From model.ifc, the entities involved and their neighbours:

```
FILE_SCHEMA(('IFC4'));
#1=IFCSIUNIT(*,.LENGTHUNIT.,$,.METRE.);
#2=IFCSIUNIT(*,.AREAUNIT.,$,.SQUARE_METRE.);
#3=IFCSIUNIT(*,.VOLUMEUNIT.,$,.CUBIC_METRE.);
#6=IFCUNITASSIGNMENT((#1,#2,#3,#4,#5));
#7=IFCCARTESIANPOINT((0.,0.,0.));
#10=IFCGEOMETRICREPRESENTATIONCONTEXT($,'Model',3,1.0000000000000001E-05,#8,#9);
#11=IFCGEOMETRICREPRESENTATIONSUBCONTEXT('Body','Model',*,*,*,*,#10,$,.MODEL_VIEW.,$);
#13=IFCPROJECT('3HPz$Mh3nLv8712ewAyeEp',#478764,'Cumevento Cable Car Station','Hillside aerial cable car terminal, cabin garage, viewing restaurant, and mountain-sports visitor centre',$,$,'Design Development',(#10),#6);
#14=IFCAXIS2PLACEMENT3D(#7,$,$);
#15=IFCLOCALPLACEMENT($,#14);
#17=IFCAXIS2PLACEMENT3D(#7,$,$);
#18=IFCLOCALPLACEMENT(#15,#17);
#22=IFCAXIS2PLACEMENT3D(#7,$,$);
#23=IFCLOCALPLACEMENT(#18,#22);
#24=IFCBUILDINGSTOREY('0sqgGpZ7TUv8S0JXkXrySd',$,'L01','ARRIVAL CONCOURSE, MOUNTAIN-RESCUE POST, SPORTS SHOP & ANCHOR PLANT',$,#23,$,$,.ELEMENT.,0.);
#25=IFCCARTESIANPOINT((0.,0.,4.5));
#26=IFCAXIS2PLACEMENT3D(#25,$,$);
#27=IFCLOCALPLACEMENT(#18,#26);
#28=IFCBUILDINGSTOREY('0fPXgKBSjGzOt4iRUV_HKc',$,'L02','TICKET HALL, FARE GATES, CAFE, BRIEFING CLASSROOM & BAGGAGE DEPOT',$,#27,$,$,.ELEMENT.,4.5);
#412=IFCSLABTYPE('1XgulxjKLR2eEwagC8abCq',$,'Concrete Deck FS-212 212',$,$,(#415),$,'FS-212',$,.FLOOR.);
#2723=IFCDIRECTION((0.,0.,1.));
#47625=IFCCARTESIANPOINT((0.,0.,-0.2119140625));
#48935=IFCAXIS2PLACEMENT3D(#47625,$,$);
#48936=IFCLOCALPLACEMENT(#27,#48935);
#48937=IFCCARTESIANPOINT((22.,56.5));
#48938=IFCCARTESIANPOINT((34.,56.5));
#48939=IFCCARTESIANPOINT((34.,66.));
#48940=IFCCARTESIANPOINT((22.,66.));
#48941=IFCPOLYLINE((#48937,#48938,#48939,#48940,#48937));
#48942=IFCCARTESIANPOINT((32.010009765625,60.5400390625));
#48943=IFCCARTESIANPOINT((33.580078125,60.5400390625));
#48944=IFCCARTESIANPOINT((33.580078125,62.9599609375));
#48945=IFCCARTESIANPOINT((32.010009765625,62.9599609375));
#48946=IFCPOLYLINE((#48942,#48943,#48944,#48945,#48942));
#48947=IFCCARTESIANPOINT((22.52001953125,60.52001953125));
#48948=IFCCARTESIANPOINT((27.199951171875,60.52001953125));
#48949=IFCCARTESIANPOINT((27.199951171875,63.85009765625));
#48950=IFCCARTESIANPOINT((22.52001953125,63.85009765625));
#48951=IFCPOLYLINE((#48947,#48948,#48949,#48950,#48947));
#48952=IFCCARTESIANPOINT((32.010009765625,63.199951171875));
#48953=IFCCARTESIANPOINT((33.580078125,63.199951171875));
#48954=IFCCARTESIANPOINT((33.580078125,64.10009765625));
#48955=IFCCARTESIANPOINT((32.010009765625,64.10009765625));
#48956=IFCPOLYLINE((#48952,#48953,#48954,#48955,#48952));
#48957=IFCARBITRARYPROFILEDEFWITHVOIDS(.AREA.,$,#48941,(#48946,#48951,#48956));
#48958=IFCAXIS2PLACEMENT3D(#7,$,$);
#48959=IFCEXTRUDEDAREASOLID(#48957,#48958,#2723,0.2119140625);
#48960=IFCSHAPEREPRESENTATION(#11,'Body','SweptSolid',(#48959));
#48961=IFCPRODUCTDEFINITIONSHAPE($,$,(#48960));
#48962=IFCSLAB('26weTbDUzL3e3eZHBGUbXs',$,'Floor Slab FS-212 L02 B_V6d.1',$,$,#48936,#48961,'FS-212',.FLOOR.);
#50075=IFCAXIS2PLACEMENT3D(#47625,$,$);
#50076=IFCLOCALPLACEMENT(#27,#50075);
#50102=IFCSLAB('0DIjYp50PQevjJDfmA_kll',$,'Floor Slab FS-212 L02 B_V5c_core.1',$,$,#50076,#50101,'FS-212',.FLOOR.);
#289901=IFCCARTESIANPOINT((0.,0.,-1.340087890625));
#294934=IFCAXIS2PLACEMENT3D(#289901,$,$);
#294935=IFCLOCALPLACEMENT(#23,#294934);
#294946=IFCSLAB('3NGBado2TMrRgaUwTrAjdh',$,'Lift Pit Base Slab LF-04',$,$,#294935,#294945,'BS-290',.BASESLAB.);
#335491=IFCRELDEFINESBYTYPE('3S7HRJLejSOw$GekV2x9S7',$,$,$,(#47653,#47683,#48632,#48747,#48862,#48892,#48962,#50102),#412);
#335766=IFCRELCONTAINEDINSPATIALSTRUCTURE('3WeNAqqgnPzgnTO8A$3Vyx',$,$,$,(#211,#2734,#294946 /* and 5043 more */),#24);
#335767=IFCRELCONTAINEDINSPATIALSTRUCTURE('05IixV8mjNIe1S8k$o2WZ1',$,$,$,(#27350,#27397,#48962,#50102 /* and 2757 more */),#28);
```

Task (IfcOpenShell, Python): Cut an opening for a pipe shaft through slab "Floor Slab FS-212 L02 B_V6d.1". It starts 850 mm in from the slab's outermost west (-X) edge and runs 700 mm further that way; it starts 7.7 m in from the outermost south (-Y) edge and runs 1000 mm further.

```python
import numpy as np
import ifcopenshell
import ifcopenshell.api.feature
import ifcopenshell.api.geometry
import ifcopenshell.api.root
import ifcopenshell.geom
import ifcopenshell.util.placement
import ifcopenshell.util.representation
import ifcopenshell.util.shape
import ifcopenshell.util.unit

model = ifcopenshell.open("model.ifc")
unit_scale = ifcopenshell.util.unit.calculate_unit_scale(model)
settings = ifcopenshell.geom.settings()


def volume(element):
    """Net volume in cubic metres, openings subtracted."""
    shape = ifcopenshell.geom.create_shape(settings, element)
    return ifcopenshell.util.shape.get_volume(shape.geometry)


slab = model.by_guid("26weTbDUzL3e3eZHBGUbXs")
before = volume(slab)

# Extent in the slab's own axes, in metres. The edges named are its -X and -Y sides.
slab_shape = ifcopenshell.geom.create_shape(settings, slab)
vertices = ifcopenshell.util.shape.get_vertices(slab_shape.geometry)
x_min, y_min, bottom = vertices.min(axis=0)
top = vertices[:, 2].max()

opening = ifcopenshell.api.root.create_entity(model, ifc_class="IfcOpeningElement", name="Pipe shaft opening", predefined_type="OPENING")
context = ifcopenshell.util.representation.get_context(model, "Model", "Body", "MODEL_VIEW")
width, depth = 0.7, 1
outline = [(0.0, 0.0), (width, 0.0), (width, depth), (0.0, depth), (0.0, 0.0)]
# Overshoot both faces by 50 mm so the cut is clean.
shape = ifcopenshell.api.geometry.add_slab_representation(
    model, context=context, depth=top - bottom + 0.1, polyline=outline
)
ifcopenshell.api.geometry.assign_representation(model, product=opening, representation=shape)

matrix = ifcopenshell.util.placement.get_local_placement(slab.ObjectPlacement)
matrix[:, 3] = matrix @ np.append(np.array([x_min + 0.85, y_min + 7.7, bottom - 0.05]) / unit_scale, 1.0)
ifcopenshell.api.geometry.edit_object_placement(model, product=opening, matrix=matrix, is_si=False)
ifcopenshell.api.feature.add_feature(model, feature=opening, element=slab)

after = volume(slab)

print(f"slab volume {before:.3f} -> {after:.3f} m3")

model.write("model_v2.ifc")
```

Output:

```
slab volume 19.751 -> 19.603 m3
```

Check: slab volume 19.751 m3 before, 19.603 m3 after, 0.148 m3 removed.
